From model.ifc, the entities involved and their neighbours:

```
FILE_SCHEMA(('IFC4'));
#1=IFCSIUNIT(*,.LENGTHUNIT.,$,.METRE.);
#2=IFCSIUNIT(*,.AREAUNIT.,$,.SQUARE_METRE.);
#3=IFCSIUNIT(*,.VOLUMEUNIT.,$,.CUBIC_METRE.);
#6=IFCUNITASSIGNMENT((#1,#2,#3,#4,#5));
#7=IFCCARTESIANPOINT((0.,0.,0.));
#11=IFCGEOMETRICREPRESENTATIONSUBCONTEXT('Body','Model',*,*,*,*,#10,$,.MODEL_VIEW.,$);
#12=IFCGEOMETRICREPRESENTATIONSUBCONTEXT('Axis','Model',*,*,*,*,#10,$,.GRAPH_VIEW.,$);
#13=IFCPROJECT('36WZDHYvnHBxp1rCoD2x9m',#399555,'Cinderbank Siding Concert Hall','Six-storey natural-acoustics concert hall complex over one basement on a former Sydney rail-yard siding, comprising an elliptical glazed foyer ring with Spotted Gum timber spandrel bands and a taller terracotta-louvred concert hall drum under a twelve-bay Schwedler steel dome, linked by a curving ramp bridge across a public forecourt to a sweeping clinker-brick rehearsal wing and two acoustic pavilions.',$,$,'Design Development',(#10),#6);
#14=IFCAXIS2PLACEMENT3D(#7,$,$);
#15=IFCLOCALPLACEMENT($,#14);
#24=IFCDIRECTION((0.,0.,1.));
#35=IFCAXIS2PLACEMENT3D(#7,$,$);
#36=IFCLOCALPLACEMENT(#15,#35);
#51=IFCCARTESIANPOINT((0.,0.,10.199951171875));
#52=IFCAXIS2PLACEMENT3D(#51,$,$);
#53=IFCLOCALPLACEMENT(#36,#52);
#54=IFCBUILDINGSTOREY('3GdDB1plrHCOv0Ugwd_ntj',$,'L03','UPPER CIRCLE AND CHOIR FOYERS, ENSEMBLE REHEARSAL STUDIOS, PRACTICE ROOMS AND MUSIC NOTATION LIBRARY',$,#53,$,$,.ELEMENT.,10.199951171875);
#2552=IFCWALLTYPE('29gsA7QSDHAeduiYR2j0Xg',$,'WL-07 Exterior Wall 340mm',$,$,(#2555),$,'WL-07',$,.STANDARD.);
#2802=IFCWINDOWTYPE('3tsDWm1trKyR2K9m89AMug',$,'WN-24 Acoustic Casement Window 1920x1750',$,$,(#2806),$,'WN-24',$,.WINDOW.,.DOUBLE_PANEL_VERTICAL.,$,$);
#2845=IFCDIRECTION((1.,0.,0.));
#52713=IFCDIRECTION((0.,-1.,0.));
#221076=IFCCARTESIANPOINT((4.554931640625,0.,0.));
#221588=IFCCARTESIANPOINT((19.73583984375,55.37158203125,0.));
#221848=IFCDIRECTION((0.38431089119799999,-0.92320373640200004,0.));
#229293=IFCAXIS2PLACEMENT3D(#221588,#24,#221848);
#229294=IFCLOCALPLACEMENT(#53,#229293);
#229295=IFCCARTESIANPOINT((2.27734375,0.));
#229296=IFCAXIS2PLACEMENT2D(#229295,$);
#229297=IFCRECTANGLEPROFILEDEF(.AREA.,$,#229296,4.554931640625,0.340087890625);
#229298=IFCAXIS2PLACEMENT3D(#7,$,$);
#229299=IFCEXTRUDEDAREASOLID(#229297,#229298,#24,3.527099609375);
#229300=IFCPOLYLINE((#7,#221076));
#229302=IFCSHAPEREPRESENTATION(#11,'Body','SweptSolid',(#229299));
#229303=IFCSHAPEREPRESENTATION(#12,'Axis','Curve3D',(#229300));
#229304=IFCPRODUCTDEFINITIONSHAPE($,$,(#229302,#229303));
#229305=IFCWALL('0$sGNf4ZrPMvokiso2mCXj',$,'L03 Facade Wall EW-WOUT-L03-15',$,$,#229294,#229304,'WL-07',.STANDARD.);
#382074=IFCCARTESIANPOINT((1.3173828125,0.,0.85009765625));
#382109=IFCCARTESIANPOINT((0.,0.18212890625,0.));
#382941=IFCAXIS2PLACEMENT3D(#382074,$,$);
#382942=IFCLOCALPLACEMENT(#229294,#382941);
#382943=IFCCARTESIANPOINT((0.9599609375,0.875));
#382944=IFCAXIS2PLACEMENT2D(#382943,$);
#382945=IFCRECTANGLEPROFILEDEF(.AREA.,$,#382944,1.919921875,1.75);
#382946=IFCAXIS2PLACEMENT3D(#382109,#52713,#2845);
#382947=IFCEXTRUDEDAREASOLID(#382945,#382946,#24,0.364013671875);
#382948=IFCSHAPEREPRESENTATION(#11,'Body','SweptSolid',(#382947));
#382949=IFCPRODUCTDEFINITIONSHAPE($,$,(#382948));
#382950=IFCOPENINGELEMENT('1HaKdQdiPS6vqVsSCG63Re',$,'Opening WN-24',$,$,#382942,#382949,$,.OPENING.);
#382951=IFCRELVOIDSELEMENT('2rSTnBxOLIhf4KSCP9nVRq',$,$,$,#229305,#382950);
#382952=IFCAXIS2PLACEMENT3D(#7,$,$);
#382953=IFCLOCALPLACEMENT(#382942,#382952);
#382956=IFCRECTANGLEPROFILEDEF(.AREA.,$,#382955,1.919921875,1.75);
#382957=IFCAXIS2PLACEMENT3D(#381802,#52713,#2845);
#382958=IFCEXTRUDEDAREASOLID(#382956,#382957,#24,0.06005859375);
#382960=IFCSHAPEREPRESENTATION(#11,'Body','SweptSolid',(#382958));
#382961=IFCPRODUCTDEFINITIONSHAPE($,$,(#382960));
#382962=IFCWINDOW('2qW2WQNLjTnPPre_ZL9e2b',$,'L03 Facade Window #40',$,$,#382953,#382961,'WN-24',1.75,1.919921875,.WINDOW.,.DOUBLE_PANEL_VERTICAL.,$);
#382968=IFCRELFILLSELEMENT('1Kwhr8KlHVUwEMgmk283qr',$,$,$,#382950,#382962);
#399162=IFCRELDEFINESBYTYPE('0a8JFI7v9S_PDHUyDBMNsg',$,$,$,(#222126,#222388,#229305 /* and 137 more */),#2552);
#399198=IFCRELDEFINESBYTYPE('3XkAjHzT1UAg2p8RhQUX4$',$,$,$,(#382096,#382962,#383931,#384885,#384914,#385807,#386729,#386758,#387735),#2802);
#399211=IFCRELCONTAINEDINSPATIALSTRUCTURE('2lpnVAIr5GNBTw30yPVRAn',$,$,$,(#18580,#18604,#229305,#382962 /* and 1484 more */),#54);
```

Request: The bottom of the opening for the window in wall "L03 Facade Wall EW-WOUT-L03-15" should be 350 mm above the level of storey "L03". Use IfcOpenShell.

```python
import numpy as np
import ifcopenshell
import ifcopenshell.api.geometry
import ifcopenshell.geom
import ifcopenshell.util.element
import ifcopenshell.util.placement
import ifcopenshell.util.shape
import ifcopenshell.util.unit

model = ifcopenshell.open("model.ifc")
unit_scale = ifcopenshell.util.unit.calculate_unit_scale(model)

window = model.by_guid("2qW2WQNLjTnPPre_ZL9e2b")
opening = window.FillsVoids[0].RelatingOpeningElement
storey = ifcopenshell.util.element.get_container(window, ifc_class="IfcBuildingStorey")
level = ifcopenshell.util.placement.get_local_placement(storey.ObjectPlacement)[2, 3]

# The opening's origin need not be at the sill, so measure its lowest point.
shape = ifcopenshell.geom.create_shape(ifcopenshell.geom.settings(), opening)
bottom = ifcopenshell.util.shape.get_shape_bottom_elevation(shape, shape.geometry) / unit_scale
dz = level + 0.35 - bottom

shift = np.array([0.0, 0.0, dz])
# The window is placed relative to its opening, so it follows when the opening moves.
matrix = ifcopenshell.util.placement.get_local_placement(opening.ObjectPlacement)
matrix[:3, 3] += shift
ifcopenshell.api.geometry.edit_object_placement(
    model, product=opening, matrix=matrix, is_si=False, should_transform_children=True
)

print(f"moved by {dz * unit_scale:+.3f} m")

model.write("model_edited.ifc")
```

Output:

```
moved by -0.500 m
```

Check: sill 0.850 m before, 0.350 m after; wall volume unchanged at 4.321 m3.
